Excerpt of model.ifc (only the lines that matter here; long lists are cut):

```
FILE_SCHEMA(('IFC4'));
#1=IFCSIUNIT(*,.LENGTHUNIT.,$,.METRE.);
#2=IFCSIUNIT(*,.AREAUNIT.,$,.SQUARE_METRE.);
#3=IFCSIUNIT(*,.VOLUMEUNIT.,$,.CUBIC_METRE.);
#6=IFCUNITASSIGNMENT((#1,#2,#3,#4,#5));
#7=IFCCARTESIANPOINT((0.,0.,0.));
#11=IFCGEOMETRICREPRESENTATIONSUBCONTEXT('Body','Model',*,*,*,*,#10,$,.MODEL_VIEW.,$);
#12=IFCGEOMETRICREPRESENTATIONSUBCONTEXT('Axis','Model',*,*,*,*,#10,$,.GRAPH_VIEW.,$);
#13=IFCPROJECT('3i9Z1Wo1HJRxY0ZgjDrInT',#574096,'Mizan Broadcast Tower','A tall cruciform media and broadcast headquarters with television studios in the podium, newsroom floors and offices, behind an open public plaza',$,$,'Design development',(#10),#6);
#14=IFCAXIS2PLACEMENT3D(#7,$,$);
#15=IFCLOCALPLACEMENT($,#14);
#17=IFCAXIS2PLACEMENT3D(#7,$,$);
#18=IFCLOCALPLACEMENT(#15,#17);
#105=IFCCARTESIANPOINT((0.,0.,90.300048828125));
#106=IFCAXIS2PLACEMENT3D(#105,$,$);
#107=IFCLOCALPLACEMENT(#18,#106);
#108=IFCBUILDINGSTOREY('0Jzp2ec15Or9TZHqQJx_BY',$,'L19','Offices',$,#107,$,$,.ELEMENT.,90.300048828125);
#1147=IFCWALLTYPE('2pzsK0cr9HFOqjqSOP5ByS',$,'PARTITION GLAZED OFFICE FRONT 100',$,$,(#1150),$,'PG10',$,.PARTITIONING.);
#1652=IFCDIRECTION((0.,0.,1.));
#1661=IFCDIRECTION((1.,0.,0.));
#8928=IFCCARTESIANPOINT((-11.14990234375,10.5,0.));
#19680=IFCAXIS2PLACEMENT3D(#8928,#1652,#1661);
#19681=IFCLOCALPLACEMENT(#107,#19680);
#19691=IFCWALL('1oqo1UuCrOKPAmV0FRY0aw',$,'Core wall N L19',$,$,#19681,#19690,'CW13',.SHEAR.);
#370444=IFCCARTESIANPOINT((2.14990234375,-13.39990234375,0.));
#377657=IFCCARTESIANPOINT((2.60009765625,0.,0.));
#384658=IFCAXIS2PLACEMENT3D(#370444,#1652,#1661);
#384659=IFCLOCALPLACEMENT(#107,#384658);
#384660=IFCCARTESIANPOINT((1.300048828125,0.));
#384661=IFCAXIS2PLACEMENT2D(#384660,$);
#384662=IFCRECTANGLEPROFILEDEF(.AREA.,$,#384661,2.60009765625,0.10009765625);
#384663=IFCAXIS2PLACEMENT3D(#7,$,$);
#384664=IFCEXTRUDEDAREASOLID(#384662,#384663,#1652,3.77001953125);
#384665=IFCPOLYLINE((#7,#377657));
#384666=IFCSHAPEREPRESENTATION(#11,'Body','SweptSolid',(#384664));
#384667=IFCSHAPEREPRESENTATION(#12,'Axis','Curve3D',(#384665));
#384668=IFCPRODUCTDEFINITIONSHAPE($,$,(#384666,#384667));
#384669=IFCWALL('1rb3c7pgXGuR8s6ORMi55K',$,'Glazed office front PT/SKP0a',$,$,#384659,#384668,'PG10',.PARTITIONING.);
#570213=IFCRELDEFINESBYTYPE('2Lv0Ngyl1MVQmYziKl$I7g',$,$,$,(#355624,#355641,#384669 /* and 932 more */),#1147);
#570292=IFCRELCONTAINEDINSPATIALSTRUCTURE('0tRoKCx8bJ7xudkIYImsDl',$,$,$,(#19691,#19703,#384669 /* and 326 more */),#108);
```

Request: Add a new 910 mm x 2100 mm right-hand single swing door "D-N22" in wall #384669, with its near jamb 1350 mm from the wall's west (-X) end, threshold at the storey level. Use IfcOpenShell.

```python
import numpy as np
import ifcopenshell
import ifcopenshell.api.feature
import ifcopenshell.api.geometry
import ifcopenshell.api.root
import ifcopenshell.api.spatial
import ifcopenshell.geom
import ifcopenshell.util.element
import ifcopenshell.util.placement
import ifcopenshell.util.representation
import ifcopenshell.util.shape
import ifcopenshell.util.unit

model = ifcopenshell.open("model.ifc")
unit_scale = ifcopenshell.util.unit.calculate_unit_scale(model)
settings = ifcopenshell.geom.settings()


def volume(element):
    """Net volume in cubic metres, openings subtracted."""
    shape = ifcopenshell.geom.create_shape(settings, element)
    return ifcopenshell.util.shape.get_volume(shape.geometry)


wall = model.by_guid("1rb3c7pgXGuR8s6ORMi55K")
storey = ifcopenshell.util.element.get_container(wall, ifc_class="IfcBuildingStorey")
context = ifcopenshell.util.representation.get_context(model, "Model", "Body", "MODEL_VIEW")
before = volume(wall)

width, height, from_end, sill = 0.91, 2.1, 1.35, 0.0  # metres

# The wall runs along its own X axis, and the end named is its -X end.
wall_shape = ifcopenshell.geom.create_shape(settings, wall)
x, y, z = ifcopenshell.util.shape.get_vertices(wall_shape.geometry).T
start = x.min() + from_end
face, thickness = float(y.min()), float(y.max() - y.min())
wall_matrix = ifcopenshell.util.placement.get_local_placement(wall.ObjectPlacement)
level = ifcopenshell.util.placement.get_local_placement(storey.ObjectPlacement)[2, 3]


def in_wall(x, y):
    """Placement at x, y metres in the wall's axes, at sill height."""
    matrix = wall_matrix.copy()
    matrix[:, 3] = wall_matrix @ np.array([x / unit_scale, y / unit_scale, 0.0, 1.0])
    matrix[2, 3] = level + sill / unit_scale
    return matrix


# Opening: a box that overshoots both wall faces by 50 mm.
opening = ifcopenshell.api.root.create_entity(model, ifc_class="IfcOpeningElement", predefined_type="OPENING")
box = ifcopenshell.api.geometry.add_wall_representation(
    model, context=context, length=width, height=height, thickness=thickness + 0.1
)
ifcopenshell.api.geometry.assign_representation(model, product=opening, representation=box)
ifcopenshell.api.geometry.edit_object_placement(model, product=opening, matrix=in_wall(start, face - 0.05), is_si=False)
ifcopenshell.api.feature.add_feature(model, feature=opening, element=wall)

door = ifcopenshell.api.root.create_entity(model, ifc_class="IfcDoor", name="D-N22", predefined_type="DOOR")
door.OverallWidth, door.OverallHeight = width / unit_scale, height / unit_scale
door.OperationType = "SINGLE_SWING_RIGHT"
body = ifcopenshell.api.geometry.add_door_representation(
    model,
    context=context,
    overall_width=door.OverallWidth,
    overall_height=door.OverallHeight,
    operation_type="SINGLE_SWING_RIGHT",
    lining_properties={"LiningDepth": thickness / unit_scale, "ThresholdDepth": thickness / unit_scale},
)
ifcopenshell.api.geometry.assign_representation(model, product=door, representation=body)
ifcopenshell.api.spatial.assign_container(model, products=[door], relating_structure=storey)
ifcopenshell.api.feature.add_filling(model, opening=opening, element=door)

# The lining spans the wall, so the door starts at the wall face.
ifcopenshell.api.geometry.edit_object_placement(model, product=door, matrix=in_wall(start, face), is_si=False)

after = volume(wall)

print(f"wall volume {before:.3f} -> {after:.3f} m3")

model.write("model_v2.ifc")
```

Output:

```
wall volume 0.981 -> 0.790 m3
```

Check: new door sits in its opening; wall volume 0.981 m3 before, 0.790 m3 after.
